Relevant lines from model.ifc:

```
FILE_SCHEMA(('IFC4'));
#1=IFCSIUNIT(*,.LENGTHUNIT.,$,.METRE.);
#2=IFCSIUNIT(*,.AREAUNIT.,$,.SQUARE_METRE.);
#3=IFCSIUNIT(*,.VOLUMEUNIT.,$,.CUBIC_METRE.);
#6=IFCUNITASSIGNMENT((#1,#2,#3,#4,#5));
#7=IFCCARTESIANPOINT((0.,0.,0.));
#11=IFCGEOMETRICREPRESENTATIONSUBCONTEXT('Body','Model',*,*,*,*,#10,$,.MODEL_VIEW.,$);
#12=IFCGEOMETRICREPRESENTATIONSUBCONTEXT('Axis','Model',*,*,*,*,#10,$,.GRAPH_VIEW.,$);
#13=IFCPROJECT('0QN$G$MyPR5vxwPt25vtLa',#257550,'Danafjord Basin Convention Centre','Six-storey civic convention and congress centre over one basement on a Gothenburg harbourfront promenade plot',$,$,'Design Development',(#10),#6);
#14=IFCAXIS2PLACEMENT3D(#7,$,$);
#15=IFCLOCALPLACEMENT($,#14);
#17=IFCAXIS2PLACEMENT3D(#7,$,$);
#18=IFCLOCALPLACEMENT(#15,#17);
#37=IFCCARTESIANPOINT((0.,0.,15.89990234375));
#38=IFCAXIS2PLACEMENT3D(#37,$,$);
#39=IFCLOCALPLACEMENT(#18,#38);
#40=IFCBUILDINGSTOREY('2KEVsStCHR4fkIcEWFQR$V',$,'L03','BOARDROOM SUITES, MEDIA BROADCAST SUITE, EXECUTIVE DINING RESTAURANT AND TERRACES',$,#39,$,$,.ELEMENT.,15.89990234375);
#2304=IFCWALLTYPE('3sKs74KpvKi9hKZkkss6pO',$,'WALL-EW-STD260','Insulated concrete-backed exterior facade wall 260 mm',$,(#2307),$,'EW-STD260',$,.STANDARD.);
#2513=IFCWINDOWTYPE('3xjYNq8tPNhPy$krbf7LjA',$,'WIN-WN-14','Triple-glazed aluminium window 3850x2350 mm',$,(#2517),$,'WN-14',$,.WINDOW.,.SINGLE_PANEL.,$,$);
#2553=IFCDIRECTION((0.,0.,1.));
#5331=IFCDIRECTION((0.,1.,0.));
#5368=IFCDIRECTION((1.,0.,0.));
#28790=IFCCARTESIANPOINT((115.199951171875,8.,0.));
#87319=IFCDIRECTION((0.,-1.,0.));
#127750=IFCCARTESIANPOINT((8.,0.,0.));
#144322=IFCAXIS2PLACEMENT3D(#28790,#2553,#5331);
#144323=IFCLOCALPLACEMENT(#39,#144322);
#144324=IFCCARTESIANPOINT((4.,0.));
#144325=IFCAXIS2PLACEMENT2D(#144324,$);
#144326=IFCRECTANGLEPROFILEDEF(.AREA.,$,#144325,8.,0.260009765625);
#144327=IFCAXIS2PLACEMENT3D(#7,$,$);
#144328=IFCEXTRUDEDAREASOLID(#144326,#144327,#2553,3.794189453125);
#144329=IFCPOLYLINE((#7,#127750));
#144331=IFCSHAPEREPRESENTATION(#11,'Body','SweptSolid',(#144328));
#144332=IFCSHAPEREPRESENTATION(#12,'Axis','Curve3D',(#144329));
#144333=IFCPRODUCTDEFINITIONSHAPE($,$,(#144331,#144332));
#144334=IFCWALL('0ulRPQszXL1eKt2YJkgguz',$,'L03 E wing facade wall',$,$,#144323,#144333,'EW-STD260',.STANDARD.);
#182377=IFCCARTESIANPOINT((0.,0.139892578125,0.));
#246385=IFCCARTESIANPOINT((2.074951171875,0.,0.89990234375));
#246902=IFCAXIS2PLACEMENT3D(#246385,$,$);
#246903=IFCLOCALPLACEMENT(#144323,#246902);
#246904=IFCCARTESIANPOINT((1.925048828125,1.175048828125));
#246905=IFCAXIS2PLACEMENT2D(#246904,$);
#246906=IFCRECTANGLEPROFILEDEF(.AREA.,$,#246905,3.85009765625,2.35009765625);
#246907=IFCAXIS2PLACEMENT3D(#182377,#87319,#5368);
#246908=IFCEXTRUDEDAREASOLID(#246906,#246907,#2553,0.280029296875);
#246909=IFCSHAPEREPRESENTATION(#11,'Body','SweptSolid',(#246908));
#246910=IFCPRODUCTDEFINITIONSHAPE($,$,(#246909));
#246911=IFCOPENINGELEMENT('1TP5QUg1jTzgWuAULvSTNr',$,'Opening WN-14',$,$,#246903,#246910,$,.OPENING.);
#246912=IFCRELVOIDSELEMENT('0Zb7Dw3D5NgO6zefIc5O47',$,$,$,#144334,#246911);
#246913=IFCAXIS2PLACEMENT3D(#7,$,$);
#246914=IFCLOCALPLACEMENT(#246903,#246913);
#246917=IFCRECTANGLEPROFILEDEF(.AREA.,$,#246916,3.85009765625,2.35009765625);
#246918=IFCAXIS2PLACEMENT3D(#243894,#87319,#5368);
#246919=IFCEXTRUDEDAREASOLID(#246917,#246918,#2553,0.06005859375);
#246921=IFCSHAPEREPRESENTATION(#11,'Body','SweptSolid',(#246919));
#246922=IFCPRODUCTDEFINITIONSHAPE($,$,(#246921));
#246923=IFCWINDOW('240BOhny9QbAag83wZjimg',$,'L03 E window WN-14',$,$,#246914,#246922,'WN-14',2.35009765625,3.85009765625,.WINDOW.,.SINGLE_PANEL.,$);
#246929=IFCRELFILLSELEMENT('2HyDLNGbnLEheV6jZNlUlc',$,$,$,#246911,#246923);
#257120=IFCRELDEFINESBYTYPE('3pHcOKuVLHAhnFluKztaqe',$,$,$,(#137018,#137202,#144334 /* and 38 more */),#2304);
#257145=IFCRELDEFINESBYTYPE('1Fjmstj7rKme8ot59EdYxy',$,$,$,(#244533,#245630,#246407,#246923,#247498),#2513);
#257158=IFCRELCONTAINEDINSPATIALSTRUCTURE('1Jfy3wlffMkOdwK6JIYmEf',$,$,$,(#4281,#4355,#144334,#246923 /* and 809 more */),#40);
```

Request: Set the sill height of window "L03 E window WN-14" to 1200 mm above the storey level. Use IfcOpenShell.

```python
import numpy as np
import ifcopenshell
import ifcopenshell.api.geometry
import ifcopenshell.geom
import ifcopenshell.util.element
import ifcopenshell.util.placement
import ifcopenshell.util.shape
import ifcopenshell.util.unit

model = ifcopenshell.open("model.ifc")
unit_scale = ifcopenshell.util.unit.calculate_unit_scale(model)

window = model.by_id(246923)
opening = window.FillsVoids[0].RelatingOpeningElement
storey = ifcopenshell.util.element.get_container(window, ifc_class="IfcBuildingStorey")
level = ifcopenshell.util.placement.get_local_placement(storey.ObjectPlacement)[2, 3]

# The opening's origin need not be at the sill, so measure its lowest point.
shape = ifcopenshell.geom.create_shape(ifcopenshell.geom.settings(), opening)
bottom = ifcopenshell.util.shape.get_shape_bottom_elevation(shape, shape.geometry) / unit_scale
dz = level + 1.2 - bottom

shift = np.array([0.0, 0.0, dz])
# The window is placed relative to its opening, so it follows when the opening moves.
matrix = ifcopenshell.util.placement.get_local_placement(opening.ObjectPlacement)
matrix[:3, 3] += shift
ifcopenshell.api.geometry.edit_object_placement(
    model, product=opening, matrix=matrix, is_si=False, should_transform_children=True
)

print(f"moved by {dz * unit_scale:+.3f} m")

model.write("model-out.ifc")
```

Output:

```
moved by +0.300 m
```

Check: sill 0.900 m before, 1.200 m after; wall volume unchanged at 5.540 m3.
